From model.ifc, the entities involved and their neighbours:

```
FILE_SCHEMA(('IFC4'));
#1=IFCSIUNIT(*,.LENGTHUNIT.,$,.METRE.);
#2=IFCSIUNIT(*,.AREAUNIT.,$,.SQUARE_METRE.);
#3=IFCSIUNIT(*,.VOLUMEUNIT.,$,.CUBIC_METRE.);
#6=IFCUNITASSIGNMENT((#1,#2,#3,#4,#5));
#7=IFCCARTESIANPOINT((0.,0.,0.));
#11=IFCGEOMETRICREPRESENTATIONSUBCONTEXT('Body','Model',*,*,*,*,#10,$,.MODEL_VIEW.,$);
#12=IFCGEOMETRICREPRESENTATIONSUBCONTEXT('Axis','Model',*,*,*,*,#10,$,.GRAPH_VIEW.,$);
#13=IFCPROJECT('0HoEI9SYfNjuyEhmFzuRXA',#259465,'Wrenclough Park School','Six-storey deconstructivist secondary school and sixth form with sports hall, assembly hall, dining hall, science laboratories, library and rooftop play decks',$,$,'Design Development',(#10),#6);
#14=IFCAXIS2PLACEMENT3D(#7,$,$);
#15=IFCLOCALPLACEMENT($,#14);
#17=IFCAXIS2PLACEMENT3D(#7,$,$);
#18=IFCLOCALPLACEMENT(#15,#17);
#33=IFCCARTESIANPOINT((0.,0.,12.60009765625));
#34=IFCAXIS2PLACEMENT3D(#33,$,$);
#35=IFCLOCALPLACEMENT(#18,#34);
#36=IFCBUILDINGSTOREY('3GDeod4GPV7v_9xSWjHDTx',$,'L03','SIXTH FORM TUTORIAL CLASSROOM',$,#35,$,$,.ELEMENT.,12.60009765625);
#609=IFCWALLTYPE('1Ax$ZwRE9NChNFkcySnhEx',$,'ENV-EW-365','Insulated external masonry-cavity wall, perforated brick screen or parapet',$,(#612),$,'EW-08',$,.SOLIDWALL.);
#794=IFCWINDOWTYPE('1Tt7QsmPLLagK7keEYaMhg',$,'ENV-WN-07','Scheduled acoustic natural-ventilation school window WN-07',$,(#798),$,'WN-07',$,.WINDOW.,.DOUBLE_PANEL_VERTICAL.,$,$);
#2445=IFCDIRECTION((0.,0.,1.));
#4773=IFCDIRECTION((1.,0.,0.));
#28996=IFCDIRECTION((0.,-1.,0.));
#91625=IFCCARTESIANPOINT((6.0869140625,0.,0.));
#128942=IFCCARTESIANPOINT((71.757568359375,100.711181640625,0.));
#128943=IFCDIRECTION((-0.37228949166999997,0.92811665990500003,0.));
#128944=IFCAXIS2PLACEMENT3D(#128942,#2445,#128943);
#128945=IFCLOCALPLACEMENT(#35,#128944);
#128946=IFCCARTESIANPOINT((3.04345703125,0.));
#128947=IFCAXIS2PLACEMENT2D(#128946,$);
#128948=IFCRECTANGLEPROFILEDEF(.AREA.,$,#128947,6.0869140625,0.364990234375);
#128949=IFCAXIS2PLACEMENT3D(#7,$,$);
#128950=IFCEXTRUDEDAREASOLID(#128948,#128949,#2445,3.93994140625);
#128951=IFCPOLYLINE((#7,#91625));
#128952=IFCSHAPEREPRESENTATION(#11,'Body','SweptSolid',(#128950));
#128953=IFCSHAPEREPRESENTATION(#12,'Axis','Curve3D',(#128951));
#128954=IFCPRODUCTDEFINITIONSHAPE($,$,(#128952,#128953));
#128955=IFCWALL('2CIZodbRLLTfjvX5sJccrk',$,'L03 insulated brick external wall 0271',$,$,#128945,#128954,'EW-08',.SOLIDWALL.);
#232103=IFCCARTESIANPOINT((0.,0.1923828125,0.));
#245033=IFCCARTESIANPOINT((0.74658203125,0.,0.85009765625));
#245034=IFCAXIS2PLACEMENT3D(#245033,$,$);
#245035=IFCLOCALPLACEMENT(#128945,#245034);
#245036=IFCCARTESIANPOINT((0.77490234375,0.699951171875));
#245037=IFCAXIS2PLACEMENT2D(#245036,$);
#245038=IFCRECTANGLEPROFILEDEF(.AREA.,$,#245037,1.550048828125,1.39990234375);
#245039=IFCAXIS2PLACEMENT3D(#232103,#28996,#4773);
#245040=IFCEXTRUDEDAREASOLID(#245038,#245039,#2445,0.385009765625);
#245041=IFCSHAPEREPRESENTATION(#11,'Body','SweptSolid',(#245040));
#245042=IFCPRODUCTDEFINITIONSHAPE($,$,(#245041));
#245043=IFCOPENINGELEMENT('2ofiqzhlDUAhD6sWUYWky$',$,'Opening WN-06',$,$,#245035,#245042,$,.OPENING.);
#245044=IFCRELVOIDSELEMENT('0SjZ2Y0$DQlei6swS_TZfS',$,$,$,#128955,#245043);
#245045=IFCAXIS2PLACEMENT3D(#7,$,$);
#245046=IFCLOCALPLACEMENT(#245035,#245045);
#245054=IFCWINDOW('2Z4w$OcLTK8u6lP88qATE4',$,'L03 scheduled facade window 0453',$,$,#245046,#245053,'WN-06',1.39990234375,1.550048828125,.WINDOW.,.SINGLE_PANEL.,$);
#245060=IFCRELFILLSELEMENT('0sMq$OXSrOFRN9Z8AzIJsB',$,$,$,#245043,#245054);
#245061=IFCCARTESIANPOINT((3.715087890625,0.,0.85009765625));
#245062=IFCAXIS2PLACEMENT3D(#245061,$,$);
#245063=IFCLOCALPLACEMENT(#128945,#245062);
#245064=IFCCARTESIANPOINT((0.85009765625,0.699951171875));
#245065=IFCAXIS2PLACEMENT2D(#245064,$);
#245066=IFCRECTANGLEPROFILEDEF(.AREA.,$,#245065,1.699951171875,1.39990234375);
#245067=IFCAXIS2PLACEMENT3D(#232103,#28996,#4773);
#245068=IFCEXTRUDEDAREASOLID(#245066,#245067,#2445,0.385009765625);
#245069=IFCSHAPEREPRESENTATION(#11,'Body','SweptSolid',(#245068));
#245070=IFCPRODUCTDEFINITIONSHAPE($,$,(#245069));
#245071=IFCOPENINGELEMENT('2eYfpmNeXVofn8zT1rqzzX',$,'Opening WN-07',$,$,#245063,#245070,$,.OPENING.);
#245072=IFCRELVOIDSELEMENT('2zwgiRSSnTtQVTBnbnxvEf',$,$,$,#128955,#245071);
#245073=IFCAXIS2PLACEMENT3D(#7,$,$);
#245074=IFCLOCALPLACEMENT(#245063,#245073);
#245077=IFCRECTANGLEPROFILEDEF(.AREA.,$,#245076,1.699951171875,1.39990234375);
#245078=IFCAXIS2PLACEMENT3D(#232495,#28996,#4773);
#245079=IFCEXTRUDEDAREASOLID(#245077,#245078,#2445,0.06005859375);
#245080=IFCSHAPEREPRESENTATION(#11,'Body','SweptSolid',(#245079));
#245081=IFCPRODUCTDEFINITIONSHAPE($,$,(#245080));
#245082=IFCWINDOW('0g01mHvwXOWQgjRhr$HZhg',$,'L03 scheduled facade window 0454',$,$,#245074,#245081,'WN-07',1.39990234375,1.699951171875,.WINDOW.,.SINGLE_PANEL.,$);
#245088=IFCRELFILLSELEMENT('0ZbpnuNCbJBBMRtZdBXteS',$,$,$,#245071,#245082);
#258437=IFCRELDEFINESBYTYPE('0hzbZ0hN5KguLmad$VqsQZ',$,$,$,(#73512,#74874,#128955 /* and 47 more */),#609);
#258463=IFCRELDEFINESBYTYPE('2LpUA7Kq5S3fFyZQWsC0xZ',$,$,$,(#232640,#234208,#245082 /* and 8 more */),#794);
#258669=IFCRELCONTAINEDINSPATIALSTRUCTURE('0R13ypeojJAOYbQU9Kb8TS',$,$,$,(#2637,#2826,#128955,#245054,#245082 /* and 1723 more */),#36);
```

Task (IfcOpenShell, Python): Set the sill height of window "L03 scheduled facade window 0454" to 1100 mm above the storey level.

```python
import numpy as np
import ifcopenshell
import ifcopenshell.api.geometry
import ifcopenshell.geom
import ifcopenshell.util.element
import ifcopenshell.util.placement
import ifcopenshell.util.shape
import ifcopenshell.util.unit

model = ifcopenshell.open("model.ifc")
unit_scale = ifcopenshell.util.unit.calculate_unit_scale(model)

window = model.by_guid("0g01mHvwXOWQgjRhr$HZhg")
opening = window.FillsVoids[0].RelatingOpeningElement
storey = ifcopenshell.util.element.get_container(window, ifc_class="IfcBuildingStorey")
level = ifcopenshell.util.placement.get_local_placement(storey.ObjectPlacement)[2, 3]

# The opening's origin need not be at the sill, so measure its lowest point.
shape = ifcopenshell.geom.create_shape(ifcopenshell.geom.settings(), opening)
bottom = ifcopenshell.util.shape.get_shape_bottom_elevation(shape, shape.geometry) / unit_scale
dz = level + 1.1 - bottom

shift = np.array([0.0, 0.0, dz])
# The window is placed relative to its opening, so it follows when the opening moves.
matrix = ifcopenshell.util.placement.get_local_placement(opening.ObjectPlacement)
matrix[:3, 3] += shift
ifcopenshell.api.geometry.edit_object_placement(
    model, product=opening, matrix=matrix, is_si=False, should_transform_children=True
)

print(f"moved by {dz * unit_scale:+.3f} m")

model.write("model-out.ifc")
```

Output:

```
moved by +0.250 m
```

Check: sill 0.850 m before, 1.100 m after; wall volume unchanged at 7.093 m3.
